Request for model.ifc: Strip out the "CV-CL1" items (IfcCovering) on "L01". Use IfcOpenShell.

First a look at what the model holds.

```python
import ifcopenshell
import ifcopenshell.util.element

model = ifcopenshell.open("model.ifc")
print(model.schema)
storey = next(s for s in model.by_type("IfcBuildingStorey") if s.Name == "L01")
coverings = [e for e in ifcopenshell.util.element.get_decomposition(storey) if e.is_a("IfcCovering")]
seen = {}
for e in coverings:
    element_type = ifcopenshell.util.element.get_type(e)
    name = element_type.Name if element_type not in (None, e) else None
    seen[name] = seen.get(name, 0) + 1
for name, count in sorted(seen.items(), key=str):
    print(count, "x", name)
```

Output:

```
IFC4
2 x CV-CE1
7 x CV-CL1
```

```python
import ifcopenshell
import ifcopenshell.api.root
import ifcopenshell.util.element

model = ifcopenshell.open("model.ifc")

storey = next(s for s in model.by_type("IfcBuildingStorey") if s.Name == "L01")
coverings = [e for e in ifcopenshell.util.element.get_decomposition(storey) if e.is_a("IfcCovering")]
targets = [e for e in coverings if (t := ifcopenshell.util.element.get_type(e)) not in (None, e) and t.Name == "CV-CL1"]

for e in targets:
    ifcopenshell.api.root.remove_product(model, product=e)
print(len(targets), "removed")

model.write("model_rev.ifc")
```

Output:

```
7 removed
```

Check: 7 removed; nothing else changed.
